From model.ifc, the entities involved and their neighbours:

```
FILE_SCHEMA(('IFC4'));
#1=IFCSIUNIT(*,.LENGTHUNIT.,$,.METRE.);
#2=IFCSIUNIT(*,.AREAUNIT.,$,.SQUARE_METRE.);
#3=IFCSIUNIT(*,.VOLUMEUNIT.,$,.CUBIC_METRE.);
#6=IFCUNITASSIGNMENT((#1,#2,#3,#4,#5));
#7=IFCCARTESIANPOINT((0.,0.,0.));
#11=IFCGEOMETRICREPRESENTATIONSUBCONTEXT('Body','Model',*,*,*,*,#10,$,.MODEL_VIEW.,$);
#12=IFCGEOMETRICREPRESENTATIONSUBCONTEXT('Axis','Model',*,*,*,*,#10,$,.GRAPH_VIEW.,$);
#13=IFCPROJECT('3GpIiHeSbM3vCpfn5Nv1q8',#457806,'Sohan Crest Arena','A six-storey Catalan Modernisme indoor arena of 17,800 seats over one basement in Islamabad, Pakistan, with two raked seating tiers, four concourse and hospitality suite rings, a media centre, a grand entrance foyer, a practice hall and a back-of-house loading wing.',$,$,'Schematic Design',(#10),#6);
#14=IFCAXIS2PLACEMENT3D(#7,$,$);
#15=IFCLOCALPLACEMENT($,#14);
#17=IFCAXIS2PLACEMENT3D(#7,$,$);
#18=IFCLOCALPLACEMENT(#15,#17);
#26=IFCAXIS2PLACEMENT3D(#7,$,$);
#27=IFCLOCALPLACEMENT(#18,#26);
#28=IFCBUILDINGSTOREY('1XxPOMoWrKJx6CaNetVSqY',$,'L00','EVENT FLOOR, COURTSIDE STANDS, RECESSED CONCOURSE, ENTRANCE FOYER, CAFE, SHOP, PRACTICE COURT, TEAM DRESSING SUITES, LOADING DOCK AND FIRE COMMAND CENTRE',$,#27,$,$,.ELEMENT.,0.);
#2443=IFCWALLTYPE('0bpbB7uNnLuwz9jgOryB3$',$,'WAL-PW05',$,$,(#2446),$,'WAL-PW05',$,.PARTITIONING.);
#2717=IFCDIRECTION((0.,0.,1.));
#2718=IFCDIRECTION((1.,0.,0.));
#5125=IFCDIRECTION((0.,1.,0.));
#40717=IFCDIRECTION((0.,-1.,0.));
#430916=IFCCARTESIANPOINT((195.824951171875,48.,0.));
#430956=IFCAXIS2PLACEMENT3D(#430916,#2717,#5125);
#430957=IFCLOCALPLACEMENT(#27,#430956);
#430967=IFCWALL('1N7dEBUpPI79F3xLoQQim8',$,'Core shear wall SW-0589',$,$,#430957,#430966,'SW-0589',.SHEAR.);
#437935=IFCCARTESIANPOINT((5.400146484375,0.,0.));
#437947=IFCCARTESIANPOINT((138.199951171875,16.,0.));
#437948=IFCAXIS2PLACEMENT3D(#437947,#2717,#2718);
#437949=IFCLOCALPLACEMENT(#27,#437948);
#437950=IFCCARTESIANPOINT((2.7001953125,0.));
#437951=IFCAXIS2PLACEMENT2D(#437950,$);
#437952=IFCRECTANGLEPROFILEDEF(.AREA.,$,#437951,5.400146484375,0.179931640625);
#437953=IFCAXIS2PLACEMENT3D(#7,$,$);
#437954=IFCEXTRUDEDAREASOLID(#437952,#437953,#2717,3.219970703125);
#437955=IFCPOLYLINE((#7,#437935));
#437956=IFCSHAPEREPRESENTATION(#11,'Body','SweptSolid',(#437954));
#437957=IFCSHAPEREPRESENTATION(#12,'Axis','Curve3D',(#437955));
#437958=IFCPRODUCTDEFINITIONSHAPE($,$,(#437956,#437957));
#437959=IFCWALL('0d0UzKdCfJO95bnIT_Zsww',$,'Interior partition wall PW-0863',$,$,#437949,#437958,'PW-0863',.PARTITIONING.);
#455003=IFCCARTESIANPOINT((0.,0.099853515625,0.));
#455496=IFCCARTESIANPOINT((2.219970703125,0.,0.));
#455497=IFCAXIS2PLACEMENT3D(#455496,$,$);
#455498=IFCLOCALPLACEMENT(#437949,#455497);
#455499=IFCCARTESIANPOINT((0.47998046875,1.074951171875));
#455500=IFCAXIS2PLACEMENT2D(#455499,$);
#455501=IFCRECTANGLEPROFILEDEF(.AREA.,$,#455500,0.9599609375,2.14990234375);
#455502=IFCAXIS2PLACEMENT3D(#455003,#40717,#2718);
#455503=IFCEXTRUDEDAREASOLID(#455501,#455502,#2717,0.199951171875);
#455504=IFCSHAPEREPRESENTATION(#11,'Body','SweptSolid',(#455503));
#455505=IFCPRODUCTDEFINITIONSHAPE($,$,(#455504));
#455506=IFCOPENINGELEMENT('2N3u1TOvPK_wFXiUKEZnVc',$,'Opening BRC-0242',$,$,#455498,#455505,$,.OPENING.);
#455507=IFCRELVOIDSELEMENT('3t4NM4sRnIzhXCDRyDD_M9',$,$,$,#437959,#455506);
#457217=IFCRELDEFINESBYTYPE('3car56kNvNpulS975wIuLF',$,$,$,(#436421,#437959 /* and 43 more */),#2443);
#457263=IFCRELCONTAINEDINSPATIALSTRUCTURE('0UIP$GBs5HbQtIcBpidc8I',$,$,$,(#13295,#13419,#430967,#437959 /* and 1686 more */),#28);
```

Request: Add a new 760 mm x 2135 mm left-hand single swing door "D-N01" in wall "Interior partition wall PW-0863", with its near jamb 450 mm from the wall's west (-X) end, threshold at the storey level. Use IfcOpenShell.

```python
import numpy as np
import ifcopenshell
import ifcopenshell.api.feature
import ifcopenshell.api.geometry
import ifcopenshell.api.root
import ifcopenshell.api.spatial
import ifcopenshell.geom
import ifcopenshell.util.element
import ifcopenshell.util.placement
import ifcopenshell.util.representation
import ifcopenshell.util.shape
import ifcopenshell.util.unit

model = ifcopenshell.open("model.ifc")
unit_scale = ifcopenshell.util.unit.calculate_unit_scale(model)
settings = ifcopenshell.geom.settings()


def volume(element):
    """Net volume in cubic metres, openings subtracted."""
    shape = ifcopenshell.geom.create_shape(settings, element)
    return ifcopenshell.util.shape.get_volume(shape.geometry)


wall = model.by_id(437959)
storey = ifcopenshell.util.element.get_container(wall, ifc_class="IfcBuildingStorey")
context = ifcopenshell.util.representation.get_context(model, "Model", "Body", "MODEL_VIEW")
before = volume(wall)

width, height, from_end, sill = 0.76, 2.135, 0.45, 0.0  # metres

# The wall runs along its own X axis, and the end named is its -X end.
wall_shape = ifcopenshell.geom.create_shape(settings, wall)
x, y, z = ifcopenshell.util.shape.get_vertices(wall_shape.geometry).T
start = x.min() + from_end
face, thickness = float(y.min()), float(y.max() - y.min())
wall_matrix = ifcopenshell.util.placement.get_local_placement(wall.ObjectPlacement)
level = ifcopenshell.util.placement.get_local_placement(storey.ObjectPlacement)[2, 3]


def in_wall(x, y):
    """Placement at x, y metres in the wall's axes, at sill height."""
    matrix = wall_matrix.copy()
    matrix[:, 3] = wall_matrix @ np.array([x / unit_scale, y / unit_scale, 0.0, 1.0])
    matrix[2, 3] = level + sill / unit_scale
    return matrix


# Opening: a box that overshoots both wall faces by 50 mm.
opening = ifcopenshell.api.root.create_entity(model, ifc_class="IfcOpeningElement", predefined_type="OPENING")
box = ifcopenshell.api.geometry.add_wall_representation(
    model, context=context, length=width, height=height, thickness=thickness + 0.1
)
ifcopenshell.api.geometry.assign_representation(model, product=opening, representation=box)
ifcopenshell.api.geometry.edit_object_placement(model, product=opening, matrix=in_wall(start, face - 0.05), is_si=False)
ifcopenshell.api.feature.add_feature(model, feature=opening, element=wall)

door = ifcopenshell.api.root.create_entity(model, ifc_class="IfcDoor", name="D-N01", predefined_type="DOOR")
door.OverallWidth, door.OverallHeight = width / unit_scale, height / unit_scale
door.OperationType = "SINGLE_SWING_LEFT"
body = ifcopenshell.api.geometry.add_door_representation(
    model,
    context=context,
    overall_width=door.OverallWidth,
    overall_height=door.OverallHeight,
    operation_type="SINGLE_SWING_LEFT",
    lining_properties={"LiningDepth": thickness / unit_scale, "ThresholdDepth": thickness / unit_scale},
)
ifcopenshell.api.geometry.assign_representation(model, product=door, representation=body)
ifcopenshell.api.spatial.assign_container(model, products=[door], relating_structure=storey)
ifcopenshell.api.feature.add_filling(model, opening=opening, element=door)

# The lining spans the wall, so the door starts at the wall face.
ifcopenshell.api.geometry.edit_object_placement(model, product=door, matrix=in_wall(start, face), is_si=False)

after = volume(wall)

print(f"wall volume {before:.3f} -> {after:.3f} m3")

model.write("model_rev.ifc")
```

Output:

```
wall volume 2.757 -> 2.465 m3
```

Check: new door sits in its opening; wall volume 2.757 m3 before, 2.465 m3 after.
